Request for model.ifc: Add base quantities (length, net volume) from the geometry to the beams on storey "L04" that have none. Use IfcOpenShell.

First a look at what the model holds.

```python
import ifcopenshell
import ifcopenshell.util.element
import ifcopenshell.util.unit

model = ifcopenshell.open("model.ifc")
print(model.schema)
for unit_type in ("LENGTHUNIT", "AREAUNIT", "VOLUMEUNIT"):
    print(unit_type, ifcopenshell.util.unit.calculate_unit_scale(model, unit_type))
storey = next(s for s in model.by_type("IfcBuildingStorey") if s.Name == "L04")
beams = [e for e in ifcopenshell.util.element.get_decomposition(storey) if e.is_a("IfcBeam")]
for e in sorted(beams, key=lambda e: e.id()):
    print(e.id(), e.is_a(), e.Name, list(ifcopenshell.util.element.get_psets(e, qtos_only=True)), sep=" | ")
```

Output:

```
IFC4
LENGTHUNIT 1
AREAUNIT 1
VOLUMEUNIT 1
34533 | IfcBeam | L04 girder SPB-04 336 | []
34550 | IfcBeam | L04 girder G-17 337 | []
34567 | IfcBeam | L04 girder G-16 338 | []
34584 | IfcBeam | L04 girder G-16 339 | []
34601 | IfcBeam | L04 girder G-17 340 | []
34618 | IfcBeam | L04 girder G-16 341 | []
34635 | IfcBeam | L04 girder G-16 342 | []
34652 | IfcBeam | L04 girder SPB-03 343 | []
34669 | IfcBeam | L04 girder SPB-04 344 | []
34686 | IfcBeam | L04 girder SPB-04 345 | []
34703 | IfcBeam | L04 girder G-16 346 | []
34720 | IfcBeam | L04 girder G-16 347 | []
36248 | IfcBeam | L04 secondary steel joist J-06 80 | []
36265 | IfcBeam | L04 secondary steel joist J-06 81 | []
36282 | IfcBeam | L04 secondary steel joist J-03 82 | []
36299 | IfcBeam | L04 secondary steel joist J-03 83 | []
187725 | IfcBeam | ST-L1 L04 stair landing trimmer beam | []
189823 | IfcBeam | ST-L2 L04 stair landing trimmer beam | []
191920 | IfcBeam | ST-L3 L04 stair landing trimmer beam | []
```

```python
import ifcopenshell
import ifcopenshell.api.pset
import ifcopenshell.geom
import ifcopenshell.util.element
import ifcopenshell.util.shape
import ifcopenshell.util.unit

model = ifcopenshell.open("model.ifc")
unit_scale = ifcopenshell.util.unit.calculate_unit_scale(model)
volume_scale = ifcopenshell.util.unit.calculate_unit_scale(model, "VOLUMEUNIT")
settings = ifcopenshell.geom.settings()

storey = next(s for s in model.by_type("IfcBuildingStorey") if s.Name == "L04")
beams = [e for e in ifcopenshell.util.element.get_decomposition(storey) if e.is_a("IfcBeam")]

for e in sorted(beams, key=lambda e: e.id()):
    if ifcopenshell.util.element.get_psets(e, qtos_only=True, should_inherit=False):
        continue
    # Geometry comes back in metres, in the element's own axes.
    shape = ifcopenshell.geom.create_shape(settings, e)
    values = {
        "Length": ifcopenshell.util.shape.get_max_xyz(shape.geometry) / unit_scale,
        "NetVolume": ifcopenshell.util.shape.get_volume(shape.geometry) / volume_scale,
    }
    qto = ifcopenshell.api.pset.add_qto(model, product=e, name="Qto_BeamBaseQuantities")
    ifcopenshell.api.pset.edit_qto(model, qto=qto, properties=values)
    print(e.id(), {k: round(v, 3) for k, v in values.items()})

model.write("model_rev.ifc")
```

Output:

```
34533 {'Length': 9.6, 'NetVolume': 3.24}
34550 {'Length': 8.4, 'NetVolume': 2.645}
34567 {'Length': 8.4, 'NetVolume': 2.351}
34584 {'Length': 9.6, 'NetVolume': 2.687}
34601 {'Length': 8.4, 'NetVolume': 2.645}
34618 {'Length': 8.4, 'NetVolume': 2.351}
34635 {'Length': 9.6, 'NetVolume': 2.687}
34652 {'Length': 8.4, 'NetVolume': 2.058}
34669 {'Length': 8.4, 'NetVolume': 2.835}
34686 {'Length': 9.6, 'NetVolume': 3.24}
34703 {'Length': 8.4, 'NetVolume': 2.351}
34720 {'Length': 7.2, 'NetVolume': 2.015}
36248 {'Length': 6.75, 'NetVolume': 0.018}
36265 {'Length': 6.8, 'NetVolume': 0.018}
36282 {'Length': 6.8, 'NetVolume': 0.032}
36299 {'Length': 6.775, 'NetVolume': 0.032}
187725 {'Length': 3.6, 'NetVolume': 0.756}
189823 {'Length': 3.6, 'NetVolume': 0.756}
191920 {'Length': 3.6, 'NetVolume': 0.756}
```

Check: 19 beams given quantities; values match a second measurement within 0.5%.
